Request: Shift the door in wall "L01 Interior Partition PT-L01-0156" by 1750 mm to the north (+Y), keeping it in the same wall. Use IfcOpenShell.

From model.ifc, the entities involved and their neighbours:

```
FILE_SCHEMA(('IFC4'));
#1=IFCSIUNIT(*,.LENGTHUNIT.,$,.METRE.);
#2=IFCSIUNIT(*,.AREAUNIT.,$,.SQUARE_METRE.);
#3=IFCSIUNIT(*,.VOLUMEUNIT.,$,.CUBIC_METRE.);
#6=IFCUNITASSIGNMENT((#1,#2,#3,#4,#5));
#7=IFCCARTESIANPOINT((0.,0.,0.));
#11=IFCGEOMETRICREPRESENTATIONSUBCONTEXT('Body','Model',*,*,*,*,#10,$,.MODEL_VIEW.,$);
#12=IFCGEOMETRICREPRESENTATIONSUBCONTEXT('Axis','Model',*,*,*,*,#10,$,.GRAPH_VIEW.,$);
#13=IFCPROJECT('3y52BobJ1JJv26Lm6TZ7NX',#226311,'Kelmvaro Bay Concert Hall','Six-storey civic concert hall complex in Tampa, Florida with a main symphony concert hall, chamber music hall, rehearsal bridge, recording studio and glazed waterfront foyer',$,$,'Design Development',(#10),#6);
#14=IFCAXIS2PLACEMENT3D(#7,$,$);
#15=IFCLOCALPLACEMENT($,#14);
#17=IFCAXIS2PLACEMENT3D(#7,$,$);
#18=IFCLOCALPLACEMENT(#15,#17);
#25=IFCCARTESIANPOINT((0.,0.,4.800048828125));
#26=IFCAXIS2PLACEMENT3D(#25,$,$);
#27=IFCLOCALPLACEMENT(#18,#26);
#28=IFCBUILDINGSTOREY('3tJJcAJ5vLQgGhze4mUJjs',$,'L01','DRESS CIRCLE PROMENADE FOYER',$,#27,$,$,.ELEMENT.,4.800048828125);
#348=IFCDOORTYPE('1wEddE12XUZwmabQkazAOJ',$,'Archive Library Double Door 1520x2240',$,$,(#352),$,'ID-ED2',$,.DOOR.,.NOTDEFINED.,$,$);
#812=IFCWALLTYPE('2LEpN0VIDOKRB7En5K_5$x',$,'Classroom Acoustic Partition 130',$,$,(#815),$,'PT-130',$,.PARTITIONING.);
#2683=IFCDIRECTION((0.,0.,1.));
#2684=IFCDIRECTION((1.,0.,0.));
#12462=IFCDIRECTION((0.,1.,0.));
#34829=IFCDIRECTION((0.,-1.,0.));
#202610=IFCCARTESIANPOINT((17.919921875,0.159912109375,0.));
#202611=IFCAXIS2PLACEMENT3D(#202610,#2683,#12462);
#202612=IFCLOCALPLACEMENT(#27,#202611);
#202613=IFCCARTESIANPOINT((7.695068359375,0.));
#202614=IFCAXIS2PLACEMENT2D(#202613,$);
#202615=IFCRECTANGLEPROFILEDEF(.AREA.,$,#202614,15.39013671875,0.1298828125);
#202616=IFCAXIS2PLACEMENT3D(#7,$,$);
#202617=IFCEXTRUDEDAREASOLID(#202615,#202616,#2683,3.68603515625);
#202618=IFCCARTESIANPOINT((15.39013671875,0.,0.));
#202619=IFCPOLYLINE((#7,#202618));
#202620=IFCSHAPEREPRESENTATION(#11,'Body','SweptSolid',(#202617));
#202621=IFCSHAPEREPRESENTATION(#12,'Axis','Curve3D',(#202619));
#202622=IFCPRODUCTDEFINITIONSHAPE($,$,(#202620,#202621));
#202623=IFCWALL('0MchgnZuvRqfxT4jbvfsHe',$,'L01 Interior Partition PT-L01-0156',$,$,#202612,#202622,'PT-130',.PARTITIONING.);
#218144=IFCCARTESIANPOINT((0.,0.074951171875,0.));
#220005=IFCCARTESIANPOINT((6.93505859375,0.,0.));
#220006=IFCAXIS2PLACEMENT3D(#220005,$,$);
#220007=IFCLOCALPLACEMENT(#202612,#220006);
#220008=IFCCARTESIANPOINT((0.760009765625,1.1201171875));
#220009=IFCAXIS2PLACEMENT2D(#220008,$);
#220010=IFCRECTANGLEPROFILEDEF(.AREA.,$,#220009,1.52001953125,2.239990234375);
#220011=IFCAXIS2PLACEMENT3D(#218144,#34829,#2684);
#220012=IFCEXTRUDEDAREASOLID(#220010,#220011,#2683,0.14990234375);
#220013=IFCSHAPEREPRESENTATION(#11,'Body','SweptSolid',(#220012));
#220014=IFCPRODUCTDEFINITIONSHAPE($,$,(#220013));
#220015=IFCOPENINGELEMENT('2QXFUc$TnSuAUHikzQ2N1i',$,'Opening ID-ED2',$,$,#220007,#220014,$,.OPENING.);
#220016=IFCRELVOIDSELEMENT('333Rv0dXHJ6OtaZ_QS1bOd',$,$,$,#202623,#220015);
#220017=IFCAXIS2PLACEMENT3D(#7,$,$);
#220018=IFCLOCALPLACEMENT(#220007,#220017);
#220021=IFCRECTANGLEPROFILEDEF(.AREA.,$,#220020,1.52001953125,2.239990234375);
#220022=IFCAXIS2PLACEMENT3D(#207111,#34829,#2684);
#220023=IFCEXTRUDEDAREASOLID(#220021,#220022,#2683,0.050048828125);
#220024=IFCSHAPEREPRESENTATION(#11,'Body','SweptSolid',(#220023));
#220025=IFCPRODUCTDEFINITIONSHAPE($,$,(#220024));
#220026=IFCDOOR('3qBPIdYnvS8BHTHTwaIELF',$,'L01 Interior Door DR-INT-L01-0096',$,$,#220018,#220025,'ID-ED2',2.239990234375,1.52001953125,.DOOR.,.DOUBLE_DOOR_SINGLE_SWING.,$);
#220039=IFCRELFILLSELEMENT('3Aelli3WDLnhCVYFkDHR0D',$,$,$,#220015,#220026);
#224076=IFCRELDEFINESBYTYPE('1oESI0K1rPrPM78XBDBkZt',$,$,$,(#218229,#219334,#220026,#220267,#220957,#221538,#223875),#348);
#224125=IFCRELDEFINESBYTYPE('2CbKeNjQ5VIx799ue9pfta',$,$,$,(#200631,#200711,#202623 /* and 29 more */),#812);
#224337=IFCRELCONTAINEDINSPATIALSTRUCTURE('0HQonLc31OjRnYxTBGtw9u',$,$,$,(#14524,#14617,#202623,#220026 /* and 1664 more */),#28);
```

```python
import ifcopenshell
import ifcopenshell.api.geometry
import ifcopenshell.util.placement
import ifcopenshell.util.unit

model = ifcopenshell.open("model.ifc")
unit_scale = ifcopenshell.util.unit.calculate_unit_scale(model)

door = model.by_id(220026)
opening = door.FillsVoids[0].RelatingOpeningElement
wall = opening.VoidsElements[0].RelatingBuildingElement

wall_matrix = ifcopenshell.util.placement.get_local_placement(wall.ObjectPlacement)
shift = wall_matrix[:3, 0] * 1.75 / unit_scale
before = ifcopenshell.util.placement.get_local_placement(door.ObjectPlacement)[:3, 3].copy()

# The door is placed relative to its opening, so it follows when the opening moves.
matrix = ifcopenshell.util.placement.get_local_placement(opening.ObjectPlacement)
matrix[:3, 3] += shift
ifcopenshell.api.geometry.edit_object_placement(
    model, product=opening, matrix=matrix, is_si=False, should_transform_children=True
)

after = ifcopenshell.util.placement.get_local_placement(door.ObjectPlacement)[:3, 3]
print("door moved by", (after - before).round(3) + 0.0)

model.write("model_rev.ifc")
```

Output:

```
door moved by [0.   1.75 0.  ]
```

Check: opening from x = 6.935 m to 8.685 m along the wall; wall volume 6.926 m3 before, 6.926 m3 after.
